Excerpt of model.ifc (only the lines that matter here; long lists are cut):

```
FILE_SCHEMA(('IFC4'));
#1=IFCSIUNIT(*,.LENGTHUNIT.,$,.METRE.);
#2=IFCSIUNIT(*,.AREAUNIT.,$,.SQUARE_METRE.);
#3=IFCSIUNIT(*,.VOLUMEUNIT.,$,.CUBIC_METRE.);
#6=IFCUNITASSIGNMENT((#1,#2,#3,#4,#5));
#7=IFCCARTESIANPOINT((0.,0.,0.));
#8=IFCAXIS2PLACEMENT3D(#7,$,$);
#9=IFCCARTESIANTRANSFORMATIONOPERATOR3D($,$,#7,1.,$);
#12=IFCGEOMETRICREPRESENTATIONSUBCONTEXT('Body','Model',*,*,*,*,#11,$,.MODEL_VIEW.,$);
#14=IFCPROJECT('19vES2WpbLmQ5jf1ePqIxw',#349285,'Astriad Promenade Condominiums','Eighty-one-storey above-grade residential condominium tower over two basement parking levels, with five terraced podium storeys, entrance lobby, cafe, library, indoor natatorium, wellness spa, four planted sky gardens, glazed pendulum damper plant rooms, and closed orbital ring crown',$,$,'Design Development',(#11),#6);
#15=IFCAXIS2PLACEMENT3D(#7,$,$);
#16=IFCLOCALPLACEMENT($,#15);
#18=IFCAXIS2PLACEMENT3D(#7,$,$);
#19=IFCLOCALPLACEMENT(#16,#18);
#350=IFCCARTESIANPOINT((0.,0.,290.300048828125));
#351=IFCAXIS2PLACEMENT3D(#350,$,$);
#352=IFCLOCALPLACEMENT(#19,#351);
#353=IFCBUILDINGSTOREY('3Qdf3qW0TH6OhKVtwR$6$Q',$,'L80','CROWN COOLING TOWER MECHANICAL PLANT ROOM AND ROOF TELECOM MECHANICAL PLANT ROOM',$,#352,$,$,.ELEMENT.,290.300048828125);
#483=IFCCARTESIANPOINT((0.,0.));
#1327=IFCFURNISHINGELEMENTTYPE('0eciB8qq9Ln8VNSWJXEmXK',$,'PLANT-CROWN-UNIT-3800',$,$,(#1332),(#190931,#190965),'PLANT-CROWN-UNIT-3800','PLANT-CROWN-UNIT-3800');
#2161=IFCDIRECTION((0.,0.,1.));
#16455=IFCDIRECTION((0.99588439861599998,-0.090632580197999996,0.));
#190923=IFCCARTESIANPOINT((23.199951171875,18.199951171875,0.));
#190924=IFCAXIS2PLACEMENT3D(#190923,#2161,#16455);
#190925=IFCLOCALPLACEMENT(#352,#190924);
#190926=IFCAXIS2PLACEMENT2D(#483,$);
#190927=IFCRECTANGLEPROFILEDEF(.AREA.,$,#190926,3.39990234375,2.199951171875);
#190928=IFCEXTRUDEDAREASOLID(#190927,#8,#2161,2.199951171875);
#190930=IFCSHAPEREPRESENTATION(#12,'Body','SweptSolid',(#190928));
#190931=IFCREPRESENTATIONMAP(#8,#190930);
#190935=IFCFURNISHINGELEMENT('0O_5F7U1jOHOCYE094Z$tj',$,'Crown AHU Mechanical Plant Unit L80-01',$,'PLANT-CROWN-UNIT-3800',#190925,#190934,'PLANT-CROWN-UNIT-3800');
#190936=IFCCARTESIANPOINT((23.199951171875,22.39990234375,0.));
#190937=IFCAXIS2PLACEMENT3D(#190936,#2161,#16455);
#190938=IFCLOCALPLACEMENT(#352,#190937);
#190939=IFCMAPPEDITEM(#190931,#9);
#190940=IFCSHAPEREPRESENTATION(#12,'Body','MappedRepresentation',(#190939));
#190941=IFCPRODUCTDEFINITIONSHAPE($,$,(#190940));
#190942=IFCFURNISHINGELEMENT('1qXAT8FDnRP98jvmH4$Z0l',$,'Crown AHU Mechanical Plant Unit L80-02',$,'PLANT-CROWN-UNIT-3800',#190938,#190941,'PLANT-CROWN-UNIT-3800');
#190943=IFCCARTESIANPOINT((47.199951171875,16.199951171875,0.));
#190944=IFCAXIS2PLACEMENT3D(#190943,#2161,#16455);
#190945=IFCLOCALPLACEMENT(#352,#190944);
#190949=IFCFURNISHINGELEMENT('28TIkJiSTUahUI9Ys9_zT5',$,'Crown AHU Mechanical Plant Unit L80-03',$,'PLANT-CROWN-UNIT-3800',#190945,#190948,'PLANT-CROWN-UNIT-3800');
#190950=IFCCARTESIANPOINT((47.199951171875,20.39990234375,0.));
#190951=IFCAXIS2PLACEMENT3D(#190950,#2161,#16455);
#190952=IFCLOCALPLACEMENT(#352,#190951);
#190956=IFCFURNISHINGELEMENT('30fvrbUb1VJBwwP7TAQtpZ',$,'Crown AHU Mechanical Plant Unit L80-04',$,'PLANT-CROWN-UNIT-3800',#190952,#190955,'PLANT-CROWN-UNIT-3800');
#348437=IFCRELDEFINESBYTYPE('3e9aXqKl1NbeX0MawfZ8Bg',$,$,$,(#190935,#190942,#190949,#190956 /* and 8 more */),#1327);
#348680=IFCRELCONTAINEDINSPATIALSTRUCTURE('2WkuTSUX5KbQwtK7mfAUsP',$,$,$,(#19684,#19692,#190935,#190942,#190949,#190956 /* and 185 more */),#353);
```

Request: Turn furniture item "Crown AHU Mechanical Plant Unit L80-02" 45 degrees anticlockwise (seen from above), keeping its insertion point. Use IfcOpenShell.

```python
import ifcopenshell
import ifcopenshell.api.geometry
import ifcopenshell.util.placement

model = ifcopenshell.open("model.ifc")

item = model.by_guid("1qXAT8FDnRP98jvmH4$Z0l")
matrix = ifcopenshell.util.placement.get_local_placement(item.ObjectPlacement)
matrix = matrix @ ifcopenshell.util.placement.rotation(45, "Z")
ifcopenshell.api.geometry.edit_object_placement(model, product=item, matrix=matrix, is_si=False)

print(ifcopenshell.util.placement.get_local_placement(item.ObjectPlacement).round(3) + 0.0)

model.write("model-out.ifc")
```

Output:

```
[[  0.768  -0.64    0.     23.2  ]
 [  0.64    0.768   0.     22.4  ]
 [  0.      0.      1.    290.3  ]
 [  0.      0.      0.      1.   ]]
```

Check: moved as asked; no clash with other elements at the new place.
